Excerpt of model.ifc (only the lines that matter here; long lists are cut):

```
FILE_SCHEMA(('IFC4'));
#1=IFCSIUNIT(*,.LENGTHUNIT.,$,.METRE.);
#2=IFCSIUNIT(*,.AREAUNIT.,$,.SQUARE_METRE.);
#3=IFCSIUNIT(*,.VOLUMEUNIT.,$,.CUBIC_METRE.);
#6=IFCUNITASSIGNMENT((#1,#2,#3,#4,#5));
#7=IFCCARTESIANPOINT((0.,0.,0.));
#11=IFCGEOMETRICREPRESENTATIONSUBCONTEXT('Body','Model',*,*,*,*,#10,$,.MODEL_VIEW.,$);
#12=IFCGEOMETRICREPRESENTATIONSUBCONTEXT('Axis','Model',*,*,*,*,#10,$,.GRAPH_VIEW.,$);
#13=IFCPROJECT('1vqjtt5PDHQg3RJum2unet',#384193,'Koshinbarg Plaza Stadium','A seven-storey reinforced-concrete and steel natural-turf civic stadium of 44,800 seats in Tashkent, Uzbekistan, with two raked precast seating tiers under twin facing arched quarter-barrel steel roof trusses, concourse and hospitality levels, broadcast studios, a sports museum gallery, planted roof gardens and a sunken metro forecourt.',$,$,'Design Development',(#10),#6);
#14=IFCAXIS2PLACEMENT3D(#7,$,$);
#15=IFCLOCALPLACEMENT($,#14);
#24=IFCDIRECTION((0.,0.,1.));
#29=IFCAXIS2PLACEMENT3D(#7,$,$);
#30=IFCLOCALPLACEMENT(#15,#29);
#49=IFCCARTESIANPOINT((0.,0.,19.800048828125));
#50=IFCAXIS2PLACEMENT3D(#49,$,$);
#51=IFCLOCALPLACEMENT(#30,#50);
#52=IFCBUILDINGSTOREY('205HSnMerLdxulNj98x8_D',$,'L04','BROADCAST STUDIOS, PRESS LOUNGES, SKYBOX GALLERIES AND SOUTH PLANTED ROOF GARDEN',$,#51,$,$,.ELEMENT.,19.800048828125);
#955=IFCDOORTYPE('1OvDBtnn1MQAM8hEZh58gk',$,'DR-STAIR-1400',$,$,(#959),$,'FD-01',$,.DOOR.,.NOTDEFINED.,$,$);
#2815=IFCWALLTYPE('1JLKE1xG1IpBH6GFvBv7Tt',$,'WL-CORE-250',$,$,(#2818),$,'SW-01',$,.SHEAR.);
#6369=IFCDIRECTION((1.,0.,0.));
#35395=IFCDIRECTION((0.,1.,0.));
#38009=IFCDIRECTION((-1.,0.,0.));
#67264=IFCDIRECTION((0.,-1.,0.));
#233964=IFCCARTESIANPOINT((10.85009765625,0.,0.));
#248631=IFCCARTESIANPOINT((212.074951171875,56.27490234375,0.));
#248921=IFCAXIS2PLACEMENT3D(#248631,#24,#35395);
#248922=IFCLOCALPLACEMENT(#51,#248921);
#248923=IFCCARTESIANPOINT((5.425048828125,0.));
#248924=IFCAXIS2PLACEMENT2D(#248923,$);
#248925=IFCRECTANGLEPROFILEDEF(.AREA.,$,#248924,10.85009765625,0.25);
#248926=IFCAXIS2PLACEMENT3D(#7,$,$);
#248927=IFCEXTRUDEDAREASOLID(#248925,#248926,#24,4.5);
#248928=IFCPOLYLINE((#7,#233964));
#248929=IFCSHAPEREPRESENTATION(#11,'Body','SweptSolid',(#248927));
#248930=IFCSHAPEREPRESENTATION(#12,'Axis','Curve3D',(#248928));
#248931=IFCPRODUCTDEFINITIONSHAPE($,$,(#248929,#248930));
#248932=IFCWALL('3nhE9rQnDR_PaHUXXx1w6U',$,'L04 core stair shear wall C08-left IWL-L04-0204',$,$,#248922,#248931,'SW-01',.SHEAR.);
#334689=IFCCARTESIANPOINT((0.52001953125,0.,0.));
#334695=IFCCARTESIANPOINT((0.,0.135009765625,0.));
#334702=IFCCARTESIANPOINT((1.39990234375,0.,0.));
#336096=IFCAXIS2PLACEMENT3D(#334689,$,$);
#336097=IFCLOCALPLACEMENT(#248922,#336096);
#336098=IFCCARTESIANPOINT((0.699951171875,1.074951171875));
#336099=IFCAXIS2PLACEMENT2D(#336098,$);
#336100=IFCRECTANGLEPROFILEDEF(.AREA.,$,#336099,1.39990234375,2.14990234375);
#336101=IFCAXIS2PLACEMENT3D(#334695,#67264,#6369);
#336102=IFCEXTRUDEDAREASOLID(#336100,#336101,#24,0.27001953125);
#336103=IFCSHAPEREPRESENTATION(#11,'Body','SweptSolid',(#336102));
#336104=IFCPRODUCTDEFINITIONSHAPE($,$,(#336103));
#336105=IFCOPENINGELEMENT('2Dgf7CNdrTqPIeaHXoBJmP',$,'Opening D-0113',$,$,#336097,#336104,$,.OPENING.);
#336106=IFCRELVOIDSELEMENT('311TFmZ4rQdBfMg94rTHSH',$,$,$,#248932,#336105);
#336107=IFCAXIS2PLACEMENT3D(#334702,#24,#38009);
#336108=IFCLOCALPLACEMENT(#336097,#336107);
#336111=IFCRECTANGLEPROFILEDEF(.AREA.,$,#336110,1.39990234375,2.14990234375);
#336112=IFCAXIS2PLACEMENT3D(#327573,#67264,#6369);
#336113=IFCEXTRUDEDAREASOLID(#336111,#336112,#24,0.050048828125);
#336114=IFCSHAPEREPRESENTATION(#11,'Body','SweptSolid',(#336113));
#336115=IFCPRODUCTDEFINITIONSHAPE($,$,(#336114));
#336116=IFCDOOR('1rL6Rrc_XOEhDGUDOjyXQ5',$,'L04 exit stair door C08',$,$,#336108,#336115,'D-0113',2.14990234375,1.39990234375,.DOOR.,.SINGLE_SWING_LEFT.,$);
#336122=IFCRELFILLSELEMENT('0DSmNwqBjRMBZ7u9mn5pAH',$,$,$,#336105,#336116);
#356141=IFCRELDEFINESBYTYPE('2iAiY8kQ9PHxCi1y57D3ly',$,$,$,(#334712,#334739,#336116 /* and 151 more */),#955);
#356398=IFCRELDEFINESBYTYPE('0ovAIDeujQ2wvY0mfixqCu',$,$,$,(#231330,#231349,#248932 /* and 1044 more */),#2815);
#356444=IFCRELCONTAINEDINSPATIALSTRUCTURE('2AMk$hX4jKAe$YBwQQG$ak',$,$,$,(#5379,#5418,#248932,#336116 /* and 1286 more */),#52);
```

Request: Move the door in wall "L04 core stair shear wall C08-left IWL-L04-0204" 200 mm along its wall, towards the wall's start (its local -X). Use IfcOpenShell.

```python
import ifcopenshell
import ifcopenshell.api.geometry
import ifcopenshell.util.placement

model = ifcopenshell.open("model.ifc")

door = model.by_guid("1rL6Rrc_XOEhDGUDOjyXQ5")
opening = door.FillsVoids[0].RelatingOpeningElement
wall = opening.VoidsElements[0].RelatingBuildingElement

wall_matrix = ifcopenshell.util.placement.get_local_placement(wall.ObjectPlacement)
shift = wall_matrix[:3, 0] * -0.2
before = ifcopenshell.util.placement.get_local_placement(door.ObjectPlacement)[:3, 3].copy()

# The door is placed relative to its opening, so it follows when the opening moves.
matrix = ifcopenshell.util.placement.get_local_placement(opening.ObjectPlacement)
matrix[:3, 3] += shift
ifcopenshell.api.geometry.edit_object_placement(
    model, product=opening, matrix=matrix, is_si=False, should_transform_children=True
)

after = ifcopenshell.util.placement.get_local_placement(door.ObjectPlacement)[:3, 3]
print("door moved by", (after - before).round(3) + 0.0)

model.write("model-out.ifc")
```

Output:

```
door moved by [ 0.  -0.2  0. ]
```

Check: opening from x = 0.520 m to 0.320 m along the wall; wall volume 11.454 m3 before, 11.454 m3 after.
